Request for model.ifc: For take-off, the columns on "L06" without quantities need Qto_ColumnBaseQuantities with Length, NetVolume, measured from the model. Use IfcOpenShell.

First a look at what the model holds.

```python
import ifcopenshell
import ifcopenshell.util.element
import ifcopenshell.util.unit

model = ifcopenshell.open("model.ifc")
print(model.schema)
for unit_type in ("LENGTHUNIT", "AREAUNIT", "VOLUMEUNIT"):
    print(unit_type, ifcopenshell.util.unit.calculate_unit_scale(model, unit_type))
storey = next(s for s in model.by_type("IfcBuildingStorey") if s.Name == "L06")
columns = [e for e in ifcopenshell.util.element.get_decomposition(storey) if e.is_a("IfcColumn")]
for e in sorted(columns, key=lambda e: e.id()):
    print(e.id(), e.is_a(), e.Name, list(ifcopenshell.util.element.get_psets(e, qtos_only=True)), sep=" | ")
```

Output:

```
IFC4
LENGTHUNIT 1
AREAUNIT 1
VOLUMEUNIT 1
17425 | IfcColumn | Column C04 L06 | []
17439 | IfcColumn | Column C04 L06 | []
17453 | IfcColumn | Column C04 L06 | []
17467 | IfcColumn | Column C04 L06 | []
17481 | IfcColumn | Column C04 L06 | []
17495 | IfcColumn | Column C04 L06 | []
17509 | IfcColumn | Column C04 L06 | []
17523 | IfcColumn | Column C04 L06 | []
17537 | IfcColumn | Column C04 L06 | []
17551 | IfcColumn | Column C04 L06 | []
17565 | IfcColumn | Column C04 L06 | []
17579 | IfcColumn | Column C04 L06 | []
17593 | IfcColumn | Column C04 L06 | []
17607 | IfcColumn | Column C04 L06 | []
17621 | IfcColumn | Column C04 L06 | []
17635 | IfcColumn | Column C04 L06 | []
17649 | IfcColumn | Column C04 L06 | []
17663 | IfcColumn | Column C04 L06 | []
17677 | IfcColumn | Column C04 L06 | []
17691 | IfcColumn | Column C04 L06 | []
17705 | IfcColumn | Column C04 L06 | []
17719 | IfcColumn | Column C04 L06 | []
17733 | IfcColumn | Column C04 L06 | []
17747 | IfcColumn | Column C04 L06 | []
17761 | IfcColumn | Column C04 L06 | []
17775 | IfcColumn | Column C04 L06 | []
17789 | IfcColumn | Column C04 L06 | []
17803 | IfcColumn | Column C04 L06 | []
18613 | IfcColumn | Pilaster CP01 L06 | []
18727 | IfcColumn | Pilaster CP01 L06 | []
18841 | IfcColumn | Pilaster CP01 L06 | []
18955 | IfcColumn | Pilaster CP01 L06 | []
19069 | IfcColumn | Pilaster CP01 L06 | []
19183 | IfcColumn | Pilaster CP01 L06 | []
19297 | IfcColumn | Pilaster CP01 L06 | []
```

```python
import ifcopenshell
import ifcopenshell.api.pset
import ifcopenshell.geom
import ifcopenshell.util.element
import ifcopenshell.util.shape
import ifcopenshell.util.unit

model = ifcopenshell.open("model.ifc")
unit_scale = ifcopenshell.util.unit.calculate_unit_scale(model)
volume_scale = ifcopenshell.util.unit.calculate_unit_scale(model, "VOLUMEUNIT")
settings = ifcopenshell.geom.settings()

storey = next(s for s in model.by_type("IfcBuildingStorey") if s.Name == "L06")
columns = [e for e in ifcopenshell.util.element.get_decomposition(storey) if e.is_a("IfcColumn")]

for e in sorted(columns, key=lambda e: e.id()):
    if ifcopenshell.util.element.get_psets(e, qtos_only=True, should_inherit=False):
        continue
    # Geometry comes back in metres, in the element's own axes.
    shape = ifcopenshell.geom.create_shape(settings, e)
    values = {
        "Length": ifcopenshell.util.shape.get_z(shape.geometry) / unit_scale,
        "NetVolume": ifcopenshell.util.shape.get_volume(shape.geometry) / volume_scale,
    }
    qto = ifcopenshell.api.pset.add_qto(model, product=e, name="Qto_ColumnBaseQuantities")
    ifcopenshell.api.pset.edit_qto(model, qto=qto, properties=values)
    print(e.id(), {k: round(v, 3) for k, v in values.items()})

model.write("model-out.ifc")
```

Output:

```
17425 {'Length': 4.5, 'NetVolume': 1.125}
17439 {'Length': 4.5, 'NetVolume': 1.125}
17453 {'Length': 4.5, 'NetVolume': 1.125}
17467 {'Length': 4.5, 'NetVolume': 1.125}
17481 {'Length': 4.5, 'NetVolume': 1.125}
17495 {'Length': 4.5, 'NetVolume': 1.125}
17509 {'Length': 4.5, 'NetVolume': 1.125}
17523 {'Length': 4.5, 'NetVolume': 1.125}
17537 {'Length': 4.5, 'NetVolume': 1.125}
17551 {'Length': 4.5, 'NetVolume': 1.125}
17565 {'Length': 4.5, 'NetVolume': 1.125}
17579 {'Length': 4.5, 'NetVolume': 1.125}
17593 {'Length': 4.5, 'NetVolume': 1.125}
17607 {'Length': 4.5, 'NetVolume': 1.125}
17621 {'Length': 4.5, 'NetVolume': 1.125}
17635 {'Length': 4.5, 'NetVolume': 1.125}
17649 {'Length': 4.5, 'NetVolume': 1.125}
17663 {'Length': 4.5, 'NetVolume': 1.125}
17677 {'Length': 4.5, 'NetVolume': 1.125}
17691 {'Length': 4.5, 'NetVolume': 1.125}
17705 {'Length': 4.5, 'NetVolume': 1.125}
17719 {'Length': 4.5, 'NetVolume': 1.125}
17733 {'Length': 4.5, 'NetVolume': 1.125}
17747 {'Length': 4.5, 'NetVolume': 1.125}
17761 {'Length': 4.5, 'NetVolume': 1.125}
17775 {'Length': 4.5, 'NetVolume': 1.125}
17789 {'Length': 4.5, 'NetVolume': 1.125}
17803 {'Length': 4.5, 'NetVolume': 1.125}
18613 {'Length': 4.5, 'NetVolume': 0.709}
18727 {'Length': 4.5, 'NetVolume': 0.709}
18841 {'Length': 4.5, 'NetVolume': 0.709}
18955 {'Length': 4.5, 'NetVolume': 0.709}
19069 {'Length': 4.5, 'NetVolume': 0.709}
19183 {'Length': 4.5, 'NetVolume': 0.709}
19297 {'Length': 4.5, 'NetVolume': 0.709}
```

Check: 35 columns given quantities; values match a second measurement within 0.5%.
